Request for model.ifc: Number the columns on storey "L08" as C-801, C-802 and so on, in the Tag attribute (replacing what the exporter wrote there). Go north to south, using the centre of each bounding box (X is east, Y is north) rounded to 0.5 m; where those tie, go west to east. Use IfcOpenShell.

First a look at what the model holds.

```python
import ifcopenshell
import ifcopenshell.util.element
import ifcopenshell.util.placement

model = ifcopenshell.open("model.ifc")
print(model.schema)
storey = next(s for s in model.by_type("IfcBuildingStorey") if s.Name == "L08")
columns = [e for e in ifcopenshell.util.element.get_decomposition(storey) if e.is_a("IfcColumn")]
for e in sorted(columns, key=lambda e: e.id()):
    origin = ifcopenshell.util.placement.get_local_placement(e.ObjectPlacement)[:3, 3]
    print(e.id(), e.Tag, e.Name, origin.round(2) + 0.0, sep=" | ")
```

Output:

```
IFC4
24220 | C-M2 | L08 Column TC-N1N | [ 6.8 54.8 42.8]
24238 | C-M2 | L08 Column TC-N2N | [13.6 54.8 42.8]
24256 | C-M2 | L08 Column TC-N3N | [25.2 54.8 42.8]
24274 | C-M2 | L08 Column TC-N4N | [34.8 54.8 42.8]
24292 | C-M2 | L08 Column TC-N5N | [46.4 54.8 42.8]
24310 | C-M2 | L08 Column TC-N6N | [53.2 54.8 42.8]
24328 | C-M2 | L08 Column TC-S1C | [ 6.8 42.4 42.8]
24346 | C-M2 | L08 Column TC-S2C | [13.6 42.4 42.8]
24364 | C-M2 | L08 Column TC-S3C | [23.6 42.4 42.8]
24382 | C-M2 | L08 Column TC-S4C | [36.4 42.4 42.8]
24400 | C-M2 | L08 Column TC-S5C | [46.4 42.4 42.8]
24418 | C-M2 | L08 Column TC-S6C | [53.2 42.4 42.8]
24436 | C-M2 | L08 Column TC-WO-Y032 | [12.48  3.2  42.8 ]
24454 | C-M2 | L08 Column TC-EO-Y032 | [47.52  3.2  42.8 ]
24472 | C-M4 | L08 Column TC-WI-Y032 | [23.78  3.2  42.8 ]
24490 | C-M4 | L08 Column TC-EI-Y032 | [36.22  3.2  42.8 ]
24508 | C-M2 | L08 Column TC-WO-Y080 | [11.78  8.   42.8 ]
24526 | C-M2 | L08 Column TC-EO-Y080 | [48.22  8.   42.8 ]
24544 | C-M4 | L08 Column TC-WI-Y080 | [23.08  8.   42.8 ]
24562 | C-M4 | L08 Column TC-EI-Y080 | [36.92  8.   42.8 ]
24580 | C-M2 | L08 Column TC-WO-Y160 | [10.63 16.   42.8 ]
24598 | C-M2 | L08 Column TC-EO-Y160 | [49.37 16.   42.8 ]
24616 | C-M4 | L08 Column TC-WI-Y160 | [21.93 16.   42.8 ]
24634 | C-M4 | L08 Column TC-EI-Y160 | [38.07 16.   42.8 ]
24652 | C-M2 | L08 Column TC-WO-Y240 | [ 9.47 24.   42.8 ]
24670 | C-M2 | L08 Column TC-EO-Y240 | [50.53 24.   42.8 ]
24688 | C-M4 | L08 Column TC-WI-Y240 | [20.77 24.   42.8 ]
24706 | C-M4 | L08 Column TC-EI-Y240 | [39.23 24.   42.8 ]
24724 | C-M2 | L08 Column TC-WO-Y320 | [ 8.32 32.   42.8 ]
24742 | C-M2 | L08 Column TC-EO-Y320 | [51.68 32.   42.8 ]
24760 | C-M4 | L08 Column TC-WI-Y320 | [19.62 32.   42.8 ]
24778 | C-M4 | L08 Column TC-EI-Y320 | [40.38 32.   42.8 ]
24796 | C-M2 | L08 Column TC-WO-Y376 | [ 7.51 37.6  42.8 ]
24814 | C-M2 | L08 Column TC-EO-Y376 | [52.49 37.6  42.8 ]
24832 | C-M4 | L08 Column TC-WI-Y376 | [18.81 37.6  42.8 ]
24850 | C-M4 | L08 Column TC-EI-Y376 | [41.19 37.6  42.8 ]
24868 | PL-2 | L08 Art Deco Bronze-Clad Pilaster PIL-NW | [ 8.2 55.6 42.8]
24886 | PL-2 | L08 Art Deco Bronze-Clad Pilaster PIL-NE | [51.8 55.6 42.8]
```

```python
import ifcopenshell
import ifcopenshell.geom
import ifcopenshell.util.element
import ifcopenshell.util.shape

model = ifcopenshell.open("model.ifc")
settings = ifcopenshell.geom.settings()
settings.set("use-world-coords", True)


def centre(element):
    shape = ifcopenshell.geom.create_shape(settings, element)
    return ifcopenshell.util.shape.get_bbox_centroid(shape.geometry)


storey = next(s for s in model.by_type("IfcBuildingStorey") if s.Name == "L08")
columns = [e for e in ifcopenshell.util.element.get_decomposition(storey) if e.is_a("IfcColumn")]

# Insertion points can sit at a corner or the storey origin, so sort by the geometry (in metres).
centres = {e: centre(e) for e in columns}
columns.sort(key=lambda e: (-round(centres[e][1] / 0.5), centres[e][0]))

for i, e in enumerate(columns, start=1):
    number = f"C-8{i:02d}"
    e.Tag = number
    print(e.id(), number)

model.write("model_v2.ifc")
```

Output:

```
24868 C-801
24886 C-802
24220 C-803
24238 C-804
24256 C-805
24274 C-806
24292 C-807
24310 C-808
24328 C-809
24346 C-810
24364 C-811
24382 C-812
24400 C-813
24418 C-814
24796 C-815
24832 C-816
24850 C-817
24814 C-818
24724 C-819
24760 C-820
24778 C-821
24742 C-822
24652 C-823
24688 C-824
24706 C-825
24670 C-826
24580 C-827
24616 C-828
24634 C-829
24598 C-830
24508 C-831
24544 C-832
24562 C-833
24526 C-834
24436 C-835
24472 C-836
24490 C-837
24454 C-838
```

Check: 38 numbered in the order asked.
